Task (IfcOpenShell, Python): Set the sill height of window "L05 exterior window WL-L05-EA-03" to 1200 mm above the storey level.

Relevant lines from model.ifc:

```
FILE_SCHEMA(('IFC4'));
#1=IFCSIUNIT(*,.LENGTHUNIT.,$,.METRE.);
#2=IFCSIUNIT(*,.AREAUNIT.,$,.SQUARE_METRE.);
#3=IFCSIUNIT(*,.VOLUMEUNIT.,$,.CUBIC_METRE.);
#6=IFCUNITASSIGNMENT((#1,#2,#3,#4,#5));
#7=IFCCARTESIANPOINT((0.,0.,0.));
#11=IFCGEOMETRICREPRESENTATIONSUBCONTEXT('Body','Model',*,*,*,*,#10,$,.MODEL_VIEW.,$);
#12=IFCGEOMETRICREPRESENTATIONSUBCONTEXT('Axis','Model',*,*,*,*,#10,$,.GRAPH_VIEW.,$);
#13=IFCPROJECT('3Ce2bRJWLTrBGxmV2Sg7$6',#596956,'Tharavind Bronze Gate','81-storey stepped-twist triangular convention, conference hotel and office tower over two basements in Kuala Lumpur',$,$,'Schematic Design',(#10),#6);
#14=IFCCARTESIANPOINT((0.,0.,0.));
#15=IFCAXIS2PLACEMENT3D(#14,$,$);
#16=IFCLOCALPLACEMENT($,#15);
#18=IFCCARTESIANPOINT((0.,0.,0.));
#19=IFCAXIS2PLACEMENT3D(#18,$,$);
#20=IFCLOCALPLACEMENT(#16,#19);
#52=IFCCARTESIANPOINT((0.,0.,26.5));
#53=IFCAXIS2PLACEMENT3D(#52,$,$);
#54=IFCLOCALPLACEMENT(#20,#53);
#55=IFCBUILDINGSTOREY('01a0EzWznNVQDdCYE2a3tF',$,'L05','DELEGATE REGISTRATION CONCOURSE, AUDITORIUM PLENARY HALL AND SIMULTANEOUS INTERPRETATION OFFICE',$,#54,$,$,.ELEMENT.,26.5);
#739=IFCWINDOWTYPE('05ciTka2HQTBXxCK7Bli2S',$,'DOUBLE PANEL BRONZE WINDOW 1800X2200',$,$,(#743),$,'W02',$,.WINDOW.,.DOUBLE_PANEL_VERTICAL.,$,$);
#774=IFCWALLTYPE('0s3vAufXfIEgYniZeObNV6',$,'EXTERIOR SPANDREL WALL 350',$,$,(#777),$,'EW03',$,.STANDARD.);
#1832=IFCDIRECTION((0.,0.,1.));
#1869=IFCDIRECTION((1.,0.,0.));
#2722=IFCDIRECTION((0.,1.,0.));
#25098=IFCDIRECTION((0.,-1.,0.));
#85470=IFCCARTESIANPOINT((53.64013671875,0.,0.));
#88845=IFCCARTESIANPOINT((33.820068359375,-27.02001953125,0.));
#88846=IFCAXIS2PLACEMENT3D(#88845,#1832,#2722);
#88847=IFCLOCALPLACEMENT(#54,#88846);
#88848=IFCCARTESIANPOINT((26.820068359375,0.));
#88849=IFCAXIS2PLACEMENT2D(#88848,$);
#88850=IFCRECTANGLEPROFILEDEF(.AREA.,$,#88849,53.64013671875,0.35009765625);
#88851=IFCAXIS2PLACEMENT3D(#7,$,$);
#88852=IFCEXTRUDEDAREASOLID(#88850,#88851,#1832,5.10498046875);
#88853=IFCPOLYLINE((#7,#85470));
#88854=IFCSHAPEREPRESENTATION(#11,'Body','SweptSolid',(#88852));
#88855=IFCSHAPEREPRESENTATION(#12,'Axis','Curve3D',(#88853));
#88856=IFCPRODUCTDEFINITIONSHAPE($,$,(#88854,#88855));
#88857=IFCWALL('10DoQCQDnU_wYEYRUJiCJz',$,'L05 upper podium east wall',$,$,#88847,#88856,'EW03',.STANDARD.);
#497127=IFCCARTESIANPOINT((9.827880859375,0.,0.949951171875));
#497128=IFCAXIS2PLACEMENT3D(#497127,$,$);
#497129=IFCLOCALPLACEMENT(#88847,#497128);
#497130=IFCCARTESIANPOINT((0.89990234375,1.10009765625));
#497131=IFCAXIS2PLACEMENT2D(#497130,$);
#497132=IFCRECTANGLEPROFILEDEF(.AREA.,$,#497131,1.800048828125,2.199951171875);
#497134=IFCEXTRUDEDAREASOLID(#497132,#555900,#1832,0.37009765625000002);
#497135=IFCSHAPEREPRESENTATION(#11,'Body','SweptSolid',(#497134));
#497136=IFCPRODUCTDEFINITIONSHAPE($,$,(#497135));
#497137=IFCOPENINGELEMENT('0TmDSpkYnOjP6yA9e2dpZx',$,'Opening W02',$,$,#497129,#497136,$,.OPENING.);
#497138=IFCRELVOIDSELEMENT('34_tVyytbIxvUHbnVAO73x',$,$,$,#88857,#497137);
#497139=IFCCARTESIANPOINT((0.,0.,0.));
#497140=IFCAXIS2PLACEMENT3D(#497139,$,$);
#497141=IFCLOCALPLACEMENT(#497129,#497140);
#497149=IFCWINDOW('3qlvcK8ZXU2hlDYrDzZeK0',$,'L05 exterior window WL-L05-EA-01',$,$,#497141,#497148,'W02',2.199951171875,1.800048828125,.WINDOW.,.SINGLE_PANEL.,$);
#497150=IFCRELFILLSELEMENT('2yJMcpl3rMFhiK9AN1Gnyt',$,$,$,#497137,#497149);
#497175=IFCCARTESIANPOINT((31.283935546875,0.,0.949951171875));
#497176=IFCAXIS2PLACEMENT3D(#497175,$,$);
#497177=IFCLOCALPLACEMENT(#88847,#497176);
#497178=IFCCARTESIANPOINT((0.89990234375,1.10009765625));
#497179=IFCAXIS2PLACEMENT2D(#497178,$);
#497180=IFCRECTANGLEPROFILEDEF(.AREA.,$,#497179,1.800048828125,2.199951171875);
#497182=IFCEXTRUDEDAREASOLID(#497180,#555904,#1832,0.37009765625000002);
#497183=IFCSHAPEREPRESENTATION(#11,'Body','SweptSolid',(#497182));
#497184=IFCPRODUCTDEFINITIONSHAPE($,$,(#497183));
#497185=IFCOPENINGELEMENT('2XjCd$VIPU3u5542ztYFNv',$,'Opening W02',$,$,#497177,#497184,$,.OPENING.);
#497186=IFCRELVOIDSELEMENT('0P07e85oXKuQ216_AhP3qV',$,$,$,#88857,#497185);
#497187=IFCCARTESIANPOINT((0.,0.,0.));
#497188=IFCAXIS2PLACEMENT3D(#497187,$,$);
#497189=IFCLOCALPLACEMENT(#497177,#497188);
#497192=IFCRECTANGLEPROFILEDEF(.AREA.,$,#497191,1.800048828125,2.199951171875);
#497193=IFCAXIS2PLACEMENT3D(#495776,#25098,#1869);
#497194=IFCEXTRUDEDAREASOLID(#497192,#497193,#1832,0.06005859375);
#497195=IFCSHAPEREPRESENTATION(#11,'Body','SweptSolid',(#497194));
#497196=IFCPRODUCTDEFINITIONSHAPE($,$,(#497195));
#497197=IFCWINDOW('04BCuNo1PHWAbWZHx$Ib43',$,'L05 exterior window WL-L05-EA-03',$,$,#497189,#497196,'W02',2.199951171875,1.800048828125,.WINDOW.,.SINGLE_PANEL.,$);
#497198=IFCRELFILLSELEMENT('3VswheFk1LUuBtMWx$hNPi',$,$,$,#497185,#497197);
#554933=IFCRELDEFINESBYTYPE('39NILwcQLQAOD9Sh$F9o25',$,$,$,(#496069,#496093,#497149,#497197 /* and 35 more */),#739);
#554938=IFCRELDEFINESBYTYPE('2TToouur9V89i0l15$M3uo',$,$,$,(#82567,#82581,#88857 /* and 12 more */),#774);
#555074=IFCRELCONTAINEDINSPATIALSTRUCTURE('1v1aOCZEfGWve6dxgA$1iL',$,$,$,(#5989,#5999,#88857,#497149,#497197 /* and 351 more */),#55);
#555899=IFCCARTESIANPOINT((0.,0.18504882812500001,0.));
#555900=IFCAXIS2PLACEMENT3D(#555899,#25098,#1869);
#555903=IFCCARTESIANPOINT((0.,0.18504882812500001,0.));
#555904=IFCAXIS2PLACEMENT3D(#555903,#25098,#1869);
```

```python
import numpy as np
import ifcopenshell
import ifcopenshell.api.geometry
import ifcopenshell.geom
import ifcopenshell.util.element
import ifcopenshell.util.placement
import ifcopenshell.util.shape
import ifcopenshell.util.unit

model = ifcopenshell.open("model.ifc")
unit_scale = ifcopenshell.util.unit.calculate_unit_scale(model)

window = model.by_guid("04BCuNo1PHWAbWZHx$Ib43")
opening = window.FillsVoids[0].RelatingOpeningElement
storey = ifcopenshell.util.element.get_container(window, ifc_class="IfcBuildingStorey")
level = ifcopenshell.util.placement.get_local_placement(storey.ObjectPlacement)[2, 3]

# The opening's origin need not be at the sill, so measure its lowest point.
shape = ifcopenshell.geom.create_shape(ifcopenshell.geom.settings(), opening)
bottom = ifcopenshell.util.shape.get_shape_bottom_elevation(shape, shape.geometry) / unit_scale
dz = level + 1.2 / unit_scale - bottom

shift = np.array([0.0, 0.0, dz])
# The window is placed relative to its opening, so it follows when the opening moves.
matrix = ifcopenshell.util.placement.get_local_placement(opening.ObjectPlacement)
matrix[:3, 3] += shift
ifcopenshell.api.geometry.edit_object_placement(
    model, product=opening, matrix=matrix, is_si=False, should_transform_children=True
)

print(f"moved by {dz * unit_scale:+.3f} m")

model.write("model_updated.ifc")
```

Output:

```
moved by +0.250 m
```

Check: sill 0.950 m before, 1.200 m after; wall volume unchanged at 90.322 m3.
